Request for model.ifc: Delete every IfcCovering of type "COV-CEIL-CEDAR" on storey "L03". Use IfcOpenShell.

First a look at what the model holds.

```python
import ifcopenshell
import ifcopenshell.util.element

model = ifcopenshell.open("model.ifc")
print(model.schema)
storey = next(s for s in model.by_type("IfcBuildingStorey") if s.Name == "L03")
coverings = [e for e in ifcopenshell.util.element.get_decomposition(storey) if e.is_a("IfcCovering")]
seen = {}
for e in coverings:
    element_type = ifcopenshell.util.element.get_type(e)
    name = element_type.Name if element_type not in (None, e) else None
    seen[name] = seen.get(name, 0) + 1
for name, count in sorted(seen.items(), key=str):
    print(count, "x", name)
```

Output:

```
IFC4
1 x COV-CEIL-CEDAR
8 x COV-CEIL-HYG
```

```python
import ifcopenshell
import ifcopenshell.api.root
import ifcopenshell.util.element

model = ifcopenshell.open("model.ifc")

storey = next(s for s in model.by_type("IfcBuildingStorey") if s.Name == "L03")
coverings = [e for e in ifcopenshell.util.element.get_decomposition(storey) if e.is_a("IfcCovering")]
targets = [e for e in coverings if (t := ifcopenshell.util.element.get_type(e)) not in (None, e) and t.Name == "COV-CEIL-CEDAR"]

for e in targets:
    ifcopenshell.api.root.remove_product(model, product=e)
print(len(targets), "removed")

model.write("model_updated.ifc")
```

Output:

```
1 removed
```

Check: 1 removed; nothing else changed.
